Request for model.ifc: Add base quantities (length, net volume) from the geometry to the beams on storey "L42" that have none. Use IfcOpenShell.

First a look at what the model holds.

```python
import ifcopenshell
import ifcopenshell.util.element
import ifcopenshell.util.unit

model = ifcopenshell.open("model.ifc")
print(model.schema)
for unit_type in ("LENGTHUNIT", "AREAUNIT", "VOLUMEUNIT"):
    print(unit_type, ifcopenshell.util.unit.calculate_unit_scale(model, unit_type))
storey = next(s for s in model.by_type("IfcBuildingStorey") if s.Name == "L42")
beams = [e for e in ifcopenshell.util.element.get_decomposition(storey) if e.is_a("IfcBeam")]
for e in sorted(beams, key=lambda e: e.id()):
    print(e.id(), e.is_a(), e.Name, list(ifcopenshell.util.element.get_psets(e, qtos_only=True)), sep=" | ")
```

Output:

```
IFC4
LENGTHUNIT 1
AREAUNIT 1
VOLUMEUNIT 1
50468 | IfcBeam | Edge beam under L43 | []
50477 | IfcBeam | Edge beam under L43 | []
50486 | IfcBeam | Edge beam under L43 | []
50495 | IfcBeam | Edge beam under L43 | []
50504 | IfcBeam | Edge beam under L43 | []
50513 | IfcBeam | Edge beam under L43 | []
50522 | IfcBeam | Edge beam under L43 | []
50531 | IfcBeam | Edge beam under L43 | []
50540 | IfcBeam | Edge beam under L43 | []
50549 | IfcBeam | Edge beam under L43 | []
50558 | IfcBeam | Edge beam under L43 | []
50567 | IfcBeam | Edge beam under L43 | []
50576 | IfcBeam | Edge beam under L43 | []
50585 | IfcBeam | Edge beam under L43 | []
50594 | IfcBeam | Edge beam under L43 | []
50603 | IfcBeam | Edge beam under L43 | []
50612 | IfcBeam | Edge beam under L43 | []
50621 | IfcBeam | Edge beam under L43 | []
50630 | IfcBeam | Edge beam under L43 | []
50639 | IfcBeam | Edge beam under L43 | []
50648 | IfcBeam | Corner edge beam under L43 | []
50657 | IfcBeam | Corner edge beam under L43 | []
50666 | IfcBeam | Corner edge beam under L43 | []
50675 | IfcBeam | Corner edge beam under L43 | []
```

```python
import ifcopenshell
import ifcopenshell.api.pset
import ifcopenshell.geom
import ifcopenshell.util.element
import ifcopenshell.util.shape
import ifcopenshell.util.unit

model = ifcopenshell.open("model.ifc")
unit_scale = ifcopenshell.util.unit.calculate_unit_scale(model)
volume_scale = ifcopenshell.util.unit.calculate_unit_scale(model, "VOLUMEUNIT")
settings = ifcopenshell.geom.settings()

storey = next(s for s in model.by_type("IfcBuildingStorey") if s.Name == "L42")
beams = [e for e in ifcopenshell.util.element.get_decomposition(storey) if e.is_a("IfcBeam")]

for e in sorted(beams, key=lambda e: e.id()):
    if ifcopenshell.util.element.get_psets(e, qtos_only=True, should_inherit=False):
        continue
    # Geometry comes back in metres, in the element's own axes.
    shape = ifcopenshell.geom.create_shape(settings, e)
    values = {
        "Length": ifcopenshell.util.shape.get_max_xyz(shape.geometry) / unit_scale,
        "NetVolume": ifcopenshell.util.shape.get_volume(shape.geometry) / volume_scale,
    }
    qto = ifcopenshell.api.pset.add_qto(model, product=e, name="Qto_BeamBaseQuantities")
    ifcopenshell.api.pset.edit_qto(model, qto=qto, properties=values)
    print(e.id(), {k: round(v, 3) for k, v in values.items()})

model.write("model-out.ifc")
```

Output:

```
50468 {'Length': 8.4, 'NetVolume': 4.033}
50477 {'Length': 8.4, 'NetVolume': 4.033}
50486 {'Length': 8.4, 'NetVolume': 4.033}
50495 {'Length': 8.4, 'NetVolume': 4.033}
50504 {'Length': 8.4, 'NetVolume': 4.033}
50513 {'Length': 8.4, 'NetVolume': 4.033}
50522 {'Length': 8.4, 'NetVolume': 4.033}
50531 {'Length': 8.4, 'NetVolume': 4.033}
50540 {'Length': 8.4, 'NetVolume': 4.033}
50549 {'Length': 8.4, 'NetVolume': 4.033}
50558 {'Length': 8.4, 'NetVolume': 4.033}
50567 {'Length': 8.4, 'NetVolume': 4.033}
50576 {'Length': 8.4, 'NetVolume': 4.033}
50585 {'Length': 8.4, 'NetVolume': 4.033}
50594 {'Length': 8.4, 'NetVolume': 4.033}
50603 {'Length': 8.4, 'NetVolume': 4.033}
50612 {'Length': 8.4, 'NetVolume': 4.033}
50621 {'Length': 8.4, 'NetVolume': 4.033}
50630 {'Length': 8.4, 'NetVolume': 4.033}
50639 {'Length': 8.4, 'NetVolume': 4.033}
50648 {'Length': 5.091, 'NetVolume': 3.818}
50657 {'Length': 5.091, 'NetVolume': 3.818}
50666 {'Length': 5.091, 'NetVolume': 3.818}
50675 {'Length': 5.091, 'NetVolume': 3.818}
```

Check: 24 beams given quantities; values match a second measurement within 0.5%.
